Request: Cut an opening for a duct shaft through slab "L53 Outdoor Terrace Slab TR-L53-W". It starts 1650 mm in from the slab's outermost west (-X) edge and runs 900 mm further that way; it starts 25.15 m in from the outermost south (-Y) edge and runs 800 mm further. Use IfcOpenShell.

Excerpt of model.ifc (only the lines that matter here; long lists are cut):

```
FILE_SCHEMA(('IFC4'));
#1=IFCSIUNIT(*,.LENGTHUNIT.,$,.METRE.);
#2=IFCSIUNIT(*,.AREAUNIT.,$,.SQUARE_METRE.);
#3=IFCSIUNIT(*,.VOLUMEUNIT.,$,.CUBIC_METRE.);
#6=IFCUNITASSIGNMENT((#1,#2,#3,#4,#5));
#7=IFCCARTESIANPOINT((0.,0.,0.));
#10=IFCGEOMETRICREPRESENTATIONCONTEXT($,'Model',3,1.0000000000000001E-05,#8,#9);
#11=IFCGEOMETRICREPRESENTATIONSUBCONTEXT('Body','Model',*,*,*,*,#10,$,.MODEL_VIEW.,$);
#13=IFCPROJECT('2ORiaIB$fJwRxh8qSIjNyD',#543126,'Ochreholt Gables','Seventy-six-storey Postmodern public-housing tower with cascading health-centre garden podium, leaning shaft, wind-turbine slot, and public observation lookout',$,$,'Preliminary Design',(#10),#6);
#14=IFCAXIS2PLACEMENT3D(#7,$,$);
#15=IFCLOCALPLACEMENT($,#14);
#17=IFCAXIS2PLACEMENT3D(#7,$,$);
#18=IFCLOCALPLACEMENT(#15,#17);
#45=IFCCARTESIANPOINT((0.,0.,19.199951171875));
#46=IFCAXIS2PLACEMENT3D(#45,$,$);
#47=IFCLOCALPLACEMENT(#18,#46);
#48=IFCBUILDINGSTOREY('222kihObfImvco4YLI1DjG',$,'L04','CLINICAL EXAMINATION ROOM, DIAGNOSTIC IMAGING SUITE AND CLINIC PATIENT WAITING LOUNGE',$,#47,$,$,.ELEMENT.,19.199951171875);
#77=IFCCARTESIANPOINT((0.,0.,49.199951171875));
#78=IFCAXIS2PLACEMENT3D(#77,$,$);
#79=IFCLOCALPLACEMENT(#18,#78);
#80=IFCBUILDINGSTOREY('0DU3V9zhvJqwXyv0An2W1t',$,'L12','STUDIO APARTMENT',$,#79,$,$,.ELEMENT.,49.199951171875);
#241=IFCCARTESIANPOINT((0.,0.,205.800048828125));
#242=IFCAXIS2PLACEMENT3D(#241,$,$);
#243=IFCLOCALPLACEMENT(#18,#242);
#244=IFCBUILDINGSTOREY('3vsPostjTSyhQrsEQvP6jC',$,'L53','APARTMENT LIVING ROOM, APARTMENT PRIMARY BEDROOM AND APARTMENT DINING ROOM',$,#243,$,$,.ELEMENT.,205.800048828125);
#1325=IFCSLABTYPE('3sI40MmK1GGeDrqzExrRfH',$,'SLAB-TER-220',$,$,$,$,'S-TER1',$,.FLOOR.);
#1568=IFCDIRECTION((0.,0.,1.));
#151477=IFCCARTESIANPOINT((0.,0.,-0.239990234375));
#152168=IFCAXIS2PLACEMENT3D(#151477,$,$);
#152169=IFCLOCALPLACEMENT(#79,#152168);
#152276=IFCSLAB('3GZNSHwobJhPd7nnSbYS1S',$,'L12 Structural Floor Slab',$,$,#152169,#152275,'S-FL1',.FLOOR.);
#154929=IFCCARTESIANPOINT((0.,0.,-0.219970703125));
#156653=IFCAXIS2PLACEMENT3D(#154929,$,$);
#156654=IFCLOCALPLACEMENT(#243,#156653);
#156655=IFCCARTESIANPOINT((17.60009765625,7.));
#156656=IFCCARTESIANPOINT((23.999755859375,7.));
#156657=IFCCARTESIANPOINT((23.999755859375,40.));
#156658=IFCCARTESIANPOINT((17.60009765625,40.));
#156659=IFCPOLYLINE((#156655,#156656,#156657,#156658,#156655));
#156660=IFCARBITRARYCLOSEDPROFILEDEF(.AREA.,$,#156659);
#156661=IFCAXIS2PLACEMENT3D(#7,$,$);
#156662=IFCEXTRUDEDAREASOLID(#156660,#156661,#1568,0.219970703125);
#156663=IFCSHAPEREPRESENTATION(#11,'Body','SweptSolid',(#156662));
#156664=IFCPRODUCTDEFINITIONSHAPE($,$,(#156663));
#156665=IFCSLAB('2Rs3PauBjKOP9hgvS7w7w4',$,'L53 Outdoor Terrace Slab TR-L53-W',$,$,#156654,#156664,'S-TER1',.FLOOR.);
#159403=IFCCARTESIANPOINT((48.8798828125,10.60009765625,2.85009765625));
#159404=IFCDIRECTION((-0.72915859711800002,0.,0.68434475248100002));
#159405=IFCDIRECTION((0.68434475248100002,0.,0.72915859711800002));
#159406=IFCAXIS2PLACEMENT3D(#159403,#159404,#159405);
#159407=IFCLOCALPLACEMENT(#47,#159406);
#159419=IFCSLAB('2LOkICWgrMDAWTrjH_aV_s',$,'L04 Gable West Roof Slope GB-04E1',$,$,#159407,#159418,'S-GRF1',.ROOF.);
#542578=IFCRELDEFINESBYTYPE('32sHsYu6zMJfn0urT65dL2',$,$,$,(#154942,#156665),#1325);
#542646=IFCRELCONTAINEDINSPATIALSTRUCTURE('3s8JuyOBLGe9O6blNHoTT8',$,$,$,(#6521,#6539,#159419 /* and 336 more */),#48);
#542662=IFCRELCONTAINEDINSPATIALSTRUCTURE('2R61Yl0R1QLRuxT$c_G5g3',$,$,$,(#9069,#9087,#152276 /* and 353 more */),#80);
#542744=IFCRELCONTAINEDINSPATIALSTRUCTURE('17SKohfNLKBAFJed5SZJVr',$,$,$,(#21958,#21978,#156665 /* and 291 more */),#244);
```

```python
import numpy as np
import ifcopenshell
import ifcopenshell.api.feature
import ifcopenshell.api.geometry
import ifcopenshell.api.root
import ifcopenshell.geom
import ifcopenshell.util.placement
import ifcopenshell.util.representation
import ifcopenshell.util.shape
import ifcopenshell.util.unit

model = ifcopenshell.open("model.ifc")
unit_scale = ifcopenshell.util.unit.calculate_unit_scale(model)
settings = ifcopenshell.geom.settings()


def volume(element):
    """Net volume in cubic metres, openings subtracted."""
    shape = ifcopenshell.geom.create_shape(settings, element)
    return ifcopenshell.util.shape.get_volume(shape.geometry)


slab = model.by_id(156665)
before = volume(slab)

# Extent in the slab's own axes, in metres. The edges named are its -X and -Y sides.
slab_shape = ifcopenshell.geom.create_shape(settings, slab)
vertices = ifcopenshell.util.shape.get_vertices(slab_shape.geometry)
x_min, y_min, bottom = vertices.min(axis=0)
top = vertices[:, 2].max()

opening = ifcopenshell.api.root.create_entity(model, ifc_class="IfcOpeningElement", name="Duct shaft opening", predefined_type="OPENING")
context = ifcopenshell.util.representation.get_context(model, "Model", "Body", "MODEL_VIEW")
width, depth = 0.9, 0.8
outline = [(0.0, 0.0), (width, 0.0), (width, depth), (0.0, depth), (0.0, 0.0)]
# Overshoot both faces by 50 mm so the cut is clean.
shape = ifcopenshell.api.geometry.add_slab_representation(
    model, context=context, depth=top - bottom + 0.1, polyline=outline
)
ifcopenshell.api.geometry.assign_representation(model, product=opening, representation=shape)

matrix = ifcopenshell.util.placement.get_local_placement(slab.ObjectPlacement)
matrix[:, 3] = matrix @ np.append(np.array([x_min + 1.65, y_min + 25.15, bottom - 0.05]) / unit_scale, 1.0)
ifcopenshell.api.geometry.edit_object_placement(model, product=opening, matrix=matrix, is_si=False)
ifcopenshell.api.feature.add_feature(model, feature=opening, element=slab)

after = volume(slab)

print(f"slab volume {before:.3f} -> {after:.3f} m3")

model.write("model_updated.ifc")
```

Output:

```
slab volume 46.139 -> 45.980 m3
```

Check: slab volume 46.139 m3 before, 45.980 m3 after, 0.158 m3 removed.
